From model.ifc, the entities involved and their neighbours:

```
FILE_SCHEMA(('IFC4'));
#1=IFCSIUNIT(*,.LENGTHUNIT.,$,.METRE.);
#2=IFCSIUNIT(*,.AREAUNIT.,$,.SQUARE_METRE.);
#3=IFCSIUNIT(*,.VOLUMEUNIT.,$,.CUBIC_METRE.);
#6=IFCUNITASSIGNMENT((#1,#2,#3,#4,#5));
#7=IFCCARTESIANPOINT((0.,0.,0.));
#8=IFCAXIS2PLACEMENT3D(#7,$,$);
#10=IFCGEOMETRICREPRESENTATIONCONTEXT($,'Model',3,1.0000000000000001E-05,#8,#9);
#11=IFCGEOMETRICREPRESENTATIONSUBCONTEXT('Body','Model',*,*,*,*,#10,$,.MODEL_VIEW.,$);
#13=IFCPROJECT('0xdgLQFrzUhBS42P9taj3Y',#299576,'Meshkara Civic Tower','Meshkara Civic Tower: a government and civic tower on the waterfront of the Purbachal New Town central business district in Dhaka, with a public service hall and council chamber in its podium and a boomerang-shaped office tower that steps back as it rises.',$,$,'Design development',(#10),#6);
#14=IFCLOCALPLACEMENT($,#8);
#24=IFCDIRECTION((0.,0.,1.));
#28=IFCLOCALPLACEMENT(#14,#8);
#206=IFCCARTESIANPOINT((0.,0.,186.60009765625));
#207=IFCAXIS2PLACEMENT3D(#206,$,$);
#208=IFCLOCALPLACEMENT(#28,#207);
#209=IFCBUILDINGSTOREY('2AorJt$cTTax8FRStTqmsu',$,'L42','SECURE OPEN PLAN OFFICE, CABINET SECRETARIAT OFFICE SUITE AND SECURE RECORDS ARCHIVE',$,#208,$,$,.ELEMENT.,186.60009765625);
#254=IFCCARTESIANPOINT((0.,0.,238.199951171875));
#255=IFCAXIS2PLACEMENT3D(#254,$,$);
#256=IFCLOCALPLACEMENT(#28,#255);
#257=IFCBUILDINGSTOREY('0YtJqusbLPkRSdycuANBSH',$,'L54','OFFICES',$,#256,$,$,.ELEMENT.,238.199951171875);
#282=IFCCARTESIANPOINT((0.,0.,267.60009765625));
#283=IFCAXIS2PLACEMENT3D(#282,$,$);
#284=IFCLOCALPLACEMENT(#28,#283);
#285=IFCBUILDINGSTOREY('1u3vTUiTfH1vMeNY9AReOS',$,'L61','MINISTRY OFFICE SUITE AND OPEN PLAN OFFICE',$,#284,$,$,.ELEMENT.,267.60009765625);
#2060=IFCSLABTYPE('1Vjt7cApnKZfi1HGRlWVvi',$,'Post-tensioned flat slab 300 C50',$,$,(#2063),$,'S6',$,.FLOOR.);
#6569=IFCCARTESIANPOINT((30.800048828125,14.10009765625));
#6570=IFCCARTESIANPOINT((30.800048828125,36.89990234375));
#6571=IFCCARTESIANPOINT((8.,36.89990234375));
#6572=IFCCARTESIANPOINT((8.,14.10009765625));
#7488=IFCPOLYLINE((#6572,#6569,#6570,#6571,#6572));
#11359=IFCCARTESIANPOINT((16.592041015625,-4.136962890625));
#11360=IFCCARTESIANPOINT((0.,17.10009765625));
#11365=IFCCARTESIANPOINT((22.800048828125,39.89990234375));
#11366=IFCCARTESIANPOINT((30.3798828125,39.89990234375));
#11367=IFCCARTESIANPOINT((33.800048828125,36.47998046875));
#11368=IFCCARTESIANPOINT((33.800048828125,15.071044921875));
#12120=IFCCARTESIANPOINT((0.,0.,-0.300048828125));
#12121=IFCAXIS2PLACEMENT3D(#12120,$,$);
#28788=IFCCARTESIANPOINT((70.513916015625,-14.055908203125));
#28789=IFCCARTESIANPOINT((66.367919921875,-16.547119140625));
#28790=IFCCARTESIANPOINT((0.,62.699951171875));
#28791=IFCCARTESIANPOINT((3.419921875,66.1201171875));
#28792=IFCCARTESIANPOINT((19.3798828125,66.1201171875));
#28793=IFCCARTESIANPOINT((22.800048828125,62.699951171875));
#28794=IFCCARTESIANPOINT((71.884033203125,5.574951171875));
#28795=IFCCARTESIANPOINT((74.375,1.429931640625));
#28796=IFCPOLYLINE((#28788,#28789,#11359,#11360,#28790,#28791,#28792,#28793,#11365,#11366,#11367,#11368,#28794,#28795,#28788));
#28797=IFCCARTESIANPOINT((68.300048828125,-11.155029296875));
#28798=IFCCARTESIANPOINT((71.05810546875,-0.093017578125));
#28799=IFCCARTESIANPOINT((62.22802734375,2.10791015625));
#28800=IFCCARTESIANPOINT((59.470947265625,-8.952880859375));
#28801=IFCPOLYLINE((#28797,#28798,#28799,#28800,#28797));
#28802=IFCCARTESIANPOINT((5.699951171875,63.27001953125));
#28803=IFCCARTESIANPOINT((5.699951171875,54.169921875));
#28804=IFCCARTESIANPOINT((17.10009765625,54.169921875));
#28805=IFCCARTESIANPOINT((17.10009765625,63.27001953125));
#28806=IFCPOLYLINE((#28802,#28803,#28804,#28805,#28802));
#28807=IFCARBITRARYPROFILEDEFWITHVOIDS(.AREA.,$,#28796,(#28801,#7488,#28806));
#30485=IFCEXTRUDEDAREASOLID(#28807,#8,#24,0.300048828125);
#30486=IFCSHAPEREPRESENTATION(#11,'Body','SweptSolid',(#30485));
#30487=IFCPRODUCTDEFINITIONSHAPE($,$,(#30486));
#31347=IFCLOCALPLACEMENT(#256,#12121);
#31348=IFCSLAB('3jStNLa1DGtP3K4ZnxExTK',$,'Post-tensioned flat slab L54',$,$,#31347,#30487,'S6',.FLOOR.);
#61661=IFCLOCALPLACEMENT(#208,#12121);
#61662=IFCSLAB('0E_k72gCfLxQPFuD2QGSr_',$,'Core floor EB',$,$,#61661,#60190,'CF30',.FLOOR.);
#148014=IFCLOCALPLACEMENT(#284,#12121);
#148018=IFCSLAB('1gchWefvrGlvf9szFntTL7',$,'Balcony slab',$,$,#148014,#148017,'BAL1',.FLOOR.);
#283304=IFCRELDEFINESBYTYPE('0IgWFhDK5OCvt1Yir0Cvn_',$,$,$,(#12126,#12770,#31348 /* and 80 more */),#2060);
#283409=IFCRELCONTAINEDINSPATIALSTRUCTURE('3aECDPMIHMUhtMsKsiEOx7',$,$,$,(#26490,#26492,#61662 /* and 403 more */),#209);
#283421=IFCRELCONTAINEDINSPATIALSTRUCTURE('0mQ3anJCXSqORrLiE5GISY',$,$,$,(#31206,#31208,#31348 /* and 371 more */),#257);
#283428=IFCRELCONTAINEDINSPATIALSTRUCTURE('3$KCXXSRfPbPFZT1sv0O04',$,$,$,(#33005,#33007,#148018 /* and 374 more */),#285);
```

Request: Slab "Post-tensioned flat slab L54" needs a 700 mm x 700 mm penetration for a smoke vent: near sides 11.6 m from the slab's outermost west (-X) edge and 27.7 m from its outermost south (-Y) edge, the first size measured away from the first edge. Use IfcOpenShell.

```python
import numpy as np
import ifcopenshell
import ifcopenshell.api.feature
import ifcopenshell.api.geometry
import ifcopenshell.api.root
import ifcopenshell.geom
import ifcopenshell.util.placement
import ifcopenshell.util.representation
import ifcopenshell.util.shape
import ifcopenshell.util.unit

model = ifcopenshell.open("model.ifc")
unit_scale = ifcopenshell.util.unit.calculate_unit_scale(model)
settings = ifcopenshell.geom.settings()


def volume(element):
    """Net volume in cubic metres, openings subtracted."""
    shape = ifcopenshell.geom.create_shape(settings, element)
    return ifcopenshell.util.shape.get_volume(shape.geometry)


slab = model.by_guid("3jStNLa1DGtP3K4ZnxExTK")
before = volume(slab)

# Extent in the slab's own axes, in metres. The edges named are its -X and -Y sides.
slab_shape = ifcopenshell.geom.create_shape(settings, slab)
vertices = ifcopenshell.util.shape.get_vertices(slab_shape.geometry)
x_min, y_min, bottom = vertices.min(axis=0)
top = vertices[:, 2].max()

opening = ifcopenshell.api.root.create_entity(model, ifc_class="IfcOpeningElement", name="Smoke vent opening", predefined_type="OPENING")
context = ifcopenshell.util.representation.get_context(model, "Model", "Body", "MODEL_VIEW")
width, depth = 0.7, 0.7
outline = [(0.0, 0.0), (width, 0.0), (width, depth), (0.0, depth), (0.0, 0.0)]
# Overshoot both faces by 50 mm so the cut is clean.
shape = ifcopenshell.api.geometry.add_slab_representation(
    model, context=context, depth=top - bottom + 0.1, polyline=outline
)
ifcopenshell.api.geometry.assign_representation(model, product=opening, representation=shape)

matrix = ifcopenshell.util.placement.get_local_placement(slab.ObjectPlacement)
matrix[:, 3] = matrix @ np.append(np.array([x_min + 11.6, y_min + 27.7, bottom - 0.05]) / unit_scale, 1.0)
ifcopenshell.api.geometry.edit_object_placement(model, product=opening, matrix=matrix, is_si=False)
ifcopenshell.api.feature.add_feature(model, feature=opening, element=slab)

after = volume(slab)

print(f"slab volume {before:.3f} -> {after:.3f} m3")

model.write("model_updated.ifc")
```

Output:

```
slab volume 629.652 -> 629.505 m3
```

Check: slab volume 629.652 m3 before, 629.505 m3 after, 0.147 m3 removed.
